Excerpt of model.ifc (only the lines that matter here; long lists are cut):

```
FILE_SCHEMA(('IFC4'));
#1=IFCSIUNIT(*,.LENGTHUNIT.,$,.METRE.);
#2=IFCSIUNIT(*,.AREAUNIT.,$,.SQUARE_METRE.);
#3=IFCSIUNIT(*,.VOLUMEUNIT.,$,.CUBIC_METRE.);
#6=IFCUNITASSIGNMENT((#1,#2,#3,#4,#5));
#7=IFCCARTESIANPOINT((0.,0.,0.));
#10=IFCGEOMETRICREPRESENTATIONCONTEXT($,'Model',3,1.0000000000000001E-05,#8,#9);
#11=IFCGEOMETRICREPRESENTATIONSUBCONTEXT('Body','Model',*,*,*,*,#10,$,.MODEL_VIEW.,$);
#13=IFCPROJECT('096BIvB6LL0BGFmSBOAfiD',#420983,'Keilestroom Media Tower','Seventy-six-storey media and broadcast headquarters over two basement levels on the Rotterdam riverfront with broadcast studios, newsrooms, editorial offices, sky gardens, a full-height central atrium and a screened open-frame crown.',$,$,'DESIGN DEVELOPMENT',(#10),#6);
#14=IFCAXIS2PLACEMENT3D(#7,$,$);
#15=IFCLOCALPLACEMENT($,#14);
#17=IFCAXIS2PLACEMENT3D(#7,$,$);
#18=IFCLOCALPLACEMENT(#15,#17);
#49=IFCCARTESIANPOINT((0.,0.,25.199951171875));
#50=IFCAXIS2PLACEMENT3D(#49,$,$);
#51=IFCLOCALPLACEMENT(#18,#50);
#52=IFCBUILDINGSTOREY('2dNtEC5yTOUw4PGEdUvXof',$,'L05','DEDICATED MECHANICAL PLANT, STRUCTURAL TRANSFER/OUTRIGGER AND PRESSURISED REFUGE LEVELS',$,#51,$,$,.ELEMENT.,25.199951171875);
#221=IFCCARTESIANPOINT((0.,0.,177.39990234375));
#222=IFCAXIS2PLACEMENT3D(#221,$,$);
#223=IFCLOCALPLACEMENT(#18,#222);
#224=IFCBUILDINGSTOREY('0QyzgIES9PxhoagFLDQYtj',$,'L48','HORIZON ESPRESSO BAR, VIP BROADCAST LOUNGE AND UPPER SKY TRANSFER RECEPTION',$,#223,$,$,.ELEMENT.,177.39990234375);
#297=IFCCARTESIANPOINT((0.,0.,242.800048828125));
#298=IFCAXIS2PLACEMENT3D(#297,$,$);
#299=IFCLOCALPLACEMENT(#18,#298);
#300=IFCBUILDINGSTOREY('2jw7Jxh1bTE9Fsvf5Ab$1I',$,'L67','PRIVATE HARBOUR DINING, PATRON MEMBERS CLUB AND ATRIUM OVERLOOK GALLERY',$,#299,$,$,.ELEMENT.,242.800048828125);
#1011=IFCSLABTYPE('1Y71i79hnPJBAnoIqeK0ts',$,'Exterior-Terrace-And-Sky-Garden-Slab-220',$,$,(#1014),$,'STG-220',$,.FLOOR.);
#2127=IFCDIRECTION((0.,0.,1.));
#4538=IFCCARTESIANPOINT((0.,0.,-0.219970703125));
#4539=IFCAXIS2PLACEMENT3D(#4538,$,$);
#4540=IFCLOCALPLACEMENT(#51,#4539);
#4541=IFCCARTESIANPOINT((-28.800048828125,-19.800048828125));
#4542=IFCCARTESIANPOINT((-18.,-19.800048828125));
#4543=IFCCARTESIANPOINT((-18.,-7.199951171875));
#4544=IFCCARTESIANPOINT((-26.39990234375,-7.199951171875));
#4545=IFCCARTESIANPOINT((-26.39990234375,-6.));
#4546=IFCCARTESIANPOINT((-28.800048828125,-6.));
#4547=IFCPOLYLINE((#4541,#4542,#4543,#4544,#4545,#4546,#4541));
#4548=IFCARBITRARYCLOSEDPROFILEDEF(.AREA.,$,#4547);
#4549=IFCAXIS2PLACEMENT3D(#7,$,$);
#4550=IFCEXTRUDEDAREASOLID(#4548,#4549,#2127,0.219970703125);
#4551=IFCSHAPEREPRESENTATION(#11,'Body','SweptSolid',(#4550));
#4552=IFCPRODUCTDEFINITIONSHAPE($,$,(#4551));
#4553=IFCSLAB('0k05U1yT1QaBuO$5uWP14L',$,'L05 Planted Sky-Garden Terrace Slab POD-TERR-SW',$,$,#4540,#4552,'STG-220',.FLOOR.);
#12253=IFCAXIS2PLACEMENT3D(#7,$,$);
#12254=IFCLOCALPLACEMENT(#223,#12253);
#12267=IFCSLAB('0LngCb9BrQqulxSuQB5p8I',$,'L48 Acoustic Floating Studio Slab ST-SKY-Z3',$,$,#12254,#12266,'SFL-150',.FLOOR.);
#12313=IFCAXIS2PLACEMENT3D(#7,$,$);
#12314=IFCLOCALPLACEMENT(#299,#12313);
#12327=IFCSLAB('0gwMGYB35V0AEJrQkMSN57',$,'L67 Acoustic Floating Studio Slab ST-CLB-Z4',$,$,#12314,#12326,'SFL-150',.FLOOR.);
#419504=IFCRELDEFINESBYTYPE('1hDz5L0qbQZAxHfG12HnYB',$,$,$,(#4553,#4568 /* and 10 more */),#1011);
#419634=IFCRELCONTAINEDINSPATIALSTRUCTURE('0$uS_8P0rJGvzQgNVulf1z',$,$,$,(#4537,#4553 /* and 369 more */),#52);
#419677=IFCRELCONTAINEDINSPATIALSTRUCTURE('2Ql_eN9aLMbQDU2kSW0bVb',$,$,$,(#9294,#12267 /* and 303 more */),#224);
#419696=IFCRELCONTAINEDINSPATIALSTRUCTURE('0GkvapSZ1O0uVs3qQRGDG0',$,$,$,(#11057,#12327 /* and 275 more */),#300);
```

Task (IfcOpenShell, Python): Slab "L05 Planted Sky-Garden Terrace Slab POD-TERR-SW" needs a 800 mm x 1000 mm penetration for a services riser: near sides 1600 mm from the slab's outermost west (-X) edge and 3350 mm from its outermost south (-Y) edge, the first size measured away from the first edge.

```python
import numpy as np
import ifcopenshell
import ifcopenshell.api.feature
import ifcopenshell.api.geometry
import ifcopenshell.api.root
import ifcopenshell.geom
import ifcopenshell.util.placement
import ifcopenshell.util.representation
import ifcopenshell.util.shape
import ifcopenshell.util.unit

model = ifcopenshell.open("model.ifc")
unit_scale = ifcopenshell.util.unit.calculate_unit_scale(model)
settings = ifcopenshell.geom.settings()


def volume(element):
    """Net volume in cubic metres, openings subtracted."""
    shape = ifcopenshell.geom.create_shape(settings, element)
    return ifcopenshell.util.shape.get_volume(shape.geometry)


slab = model.by_guid("0k05U1yT1QaBuO$5uWP14L")
before = volume(slab)

# Extent in the slab's own axes, in metres. The edges named are its -X and -Y sides.
slab_shape = ifcopenshell.geom.create_shape(settings, slab)
vertices = ifcopenshell.util.shape.get_vertices(slab_shape.geometry)
x_min, y_min, bottom = vertices.min(axis=0)
top = vertices[:, 2].max()

opening = ifcopenshell.api.root.create_entity(model, ifc_class="IfcOpeningElement", name="Services riser opening", predefined_type="OPENING")
context = ifcopenshell.util.representation.get_context(model, "Model", "Body", "MODEL_VIEW")
width, depth = 0.8, 1
outline = [(0.0, 0.0), (width, 0.0), (width, depth), (0.0, depth), (0.0, 0.0)]
# Overshoot both faces by 50 mm so the cut is clean.
shape = ifcopenshell.api.geometry.add_slab_representation(
    model, context=context, depth=top - bottom + 0.1, polyline=outline
)
ifcopenshell.api.geometry.assign_representation(model, product=opening, representation=shape)

matrix = ifcopenshell.util.placement.get_local_placement(slab.ObjectPlacement)
matrix[:, 3] = matrix @ np.append(np.array([x_min + 1.6, y_min + 3.35, bottom - 0.05]) / unit_scale, 1.0)
ifcopenshell.api.geometry.edit_object_placement(model, product=opening, matrix=matrix, is_si=False)
ifcopenshell.api.feature.add_feature(model, feature=opening, element=slab)

after = volume(slab)

print(f"slab volume {before:.3f} -> {after:.3f} m3")

model.write("model-out.ifc")
```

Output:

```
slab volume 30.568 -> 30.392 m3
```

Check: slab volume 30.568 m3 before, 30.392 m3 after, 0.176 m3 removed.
